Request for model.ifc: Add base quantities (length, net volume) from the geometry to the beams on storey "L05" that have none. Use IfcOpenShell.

First a look at what the model holds.

```python
import ifcopenshell
import ifcopenshell.util.element
import ifcopenshell.util.unit

model = ifcopenshell.open("model.ifc")
print(model.schema)
for unit_type in ("LENGTHUNIT", "AREAUNIT", "VOLUMEUNIT"):
    print(unit_type, ifcopenshell.util.unit.calculate_unit_scale(model, unit_type))
storey = next(s for s in model.by_type("IfcBuildingStorey") if s.Name == "L05")
beams = [e for e in ifcopenshell.util.element.get_decomposition(storey) if e.is_a("IfcBeam")]
for e in sorted(beams, key=lambda e: e.id()):
    print(e.id(), e.is_a(), e.Name, list(ifcopenshell.util.element.get_psets(e, qtos_only=True)), sep=" | ")
```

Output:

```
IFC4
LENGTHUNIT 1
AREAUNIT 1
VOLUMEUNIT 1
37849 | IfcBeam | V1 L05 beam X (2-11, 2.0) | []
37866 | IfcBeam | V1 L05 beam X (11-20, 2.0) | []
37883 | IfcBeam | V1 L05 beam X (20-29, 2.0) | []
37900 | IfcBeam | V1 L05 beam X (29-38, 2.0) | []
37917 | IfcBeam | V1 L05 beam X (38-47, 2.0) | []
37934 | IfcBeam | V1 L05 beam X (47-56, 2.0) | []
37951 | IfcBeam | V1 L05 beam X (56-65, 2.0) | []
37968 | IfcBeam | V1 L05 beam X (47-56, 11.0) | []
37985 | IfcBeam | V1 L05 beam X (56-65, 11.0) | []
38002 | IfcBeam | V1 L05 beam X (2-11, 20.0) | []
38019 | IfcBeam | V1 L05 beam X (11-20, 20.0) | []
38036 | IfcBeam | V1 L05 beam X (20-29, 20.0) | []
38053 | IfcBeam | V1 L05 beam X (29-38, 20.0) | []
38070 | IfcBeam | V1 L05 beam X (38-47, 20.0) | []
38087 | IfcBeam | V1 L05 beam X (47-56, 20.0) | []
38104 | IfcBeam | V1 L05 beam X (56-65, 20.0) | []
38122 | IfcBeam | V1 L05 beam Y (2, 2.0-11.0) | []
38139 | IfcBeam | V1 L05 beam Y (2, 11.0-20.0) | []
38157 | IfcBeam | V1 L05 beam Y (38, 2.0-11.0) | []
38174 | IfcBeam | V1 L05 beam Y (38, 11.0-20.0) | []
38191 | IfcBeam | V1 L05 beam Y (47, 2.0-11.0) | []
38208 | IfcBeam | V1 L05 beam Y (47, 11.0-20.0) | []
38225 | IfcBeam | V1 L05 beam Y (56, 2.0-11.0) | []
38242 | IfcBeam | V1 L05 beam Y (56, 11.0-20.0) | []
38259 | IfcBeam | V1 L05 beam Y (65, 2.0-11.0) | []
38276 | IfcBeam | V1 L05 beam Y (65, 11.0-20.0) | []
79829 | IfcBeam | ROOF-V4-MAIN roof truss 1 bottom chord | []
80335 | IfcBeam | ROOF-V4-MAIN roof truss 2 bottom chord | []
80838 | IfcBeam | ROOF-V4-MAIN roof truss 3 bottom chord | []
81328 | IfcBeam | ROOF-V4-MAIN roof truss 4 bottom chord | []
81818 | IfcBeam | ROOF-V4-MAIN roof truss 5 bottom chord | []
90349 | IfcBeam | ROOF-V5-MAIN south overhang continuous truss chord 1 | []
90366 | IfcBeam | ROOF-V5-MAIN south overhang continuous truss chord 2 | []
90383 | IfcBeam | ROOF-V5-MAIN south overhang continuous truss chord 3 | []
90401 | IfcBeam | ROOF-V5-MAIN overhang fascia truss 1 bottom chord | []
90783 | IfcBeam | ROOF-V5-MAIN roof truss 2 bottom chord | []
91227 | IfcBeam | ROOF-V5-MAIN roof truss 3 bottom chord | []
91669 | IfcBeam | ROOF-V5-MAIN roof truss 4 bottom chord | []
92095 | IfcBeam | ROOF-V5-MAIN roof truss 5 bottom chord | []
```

```python
import ifcopenshell
import ifcopenshell.api.pset
import ifcopenshell.geom
import ifcopenshell.util.element
import ifcopenshell.util.shape
import ifcopenshell.util.unit

model = ifcopenshell.open("model.ifc")
unit_scale = ifcopenshell.util.unit.calculate_unit_scale(model)
volume_scale = ifcopenshell.util.unit.calculate_unit_scale(model, "VOLUMEUNIT")
settings = ifcopenshell.geom.settings()

storey = next(s for s in model.by_type("IfcBuildingStorey") if s.Name == "L05")
beams = [e for e in ifcopenshell.util.element.get_decomposition(storey) if e.is_a("IfcBeam")]

for e in sorted(beams, key=lambda e: e.id()):
    if ifcopenshell.util.element.get_psets(e, qtos_only=True, should_inherit=False):
        continue
    # Geometry comes back in metres, in the element's own axes.
    shape = ifcopenshell.geom.create_shape(settings, e)
    values = {
        "Length": ifcopenshell.util.shape.get_max_xyz(shape.geometry) / unit_scale,
        "NetVolume": ifcopenshell.util.shape.get_volume(shape.geometry) / volume_scale,
    }
    qto = ifcopenshell.api.pset.add_qto(model, product=e, name="Qto_BeamBaseQuantities")
    ifcopenshell.api.pset.edit_qto(model, qto=qto, properties=values)
    print(e.id(), {k: round(v, 3) for k, v in values.items()})

model.write("model-out.ifc")
```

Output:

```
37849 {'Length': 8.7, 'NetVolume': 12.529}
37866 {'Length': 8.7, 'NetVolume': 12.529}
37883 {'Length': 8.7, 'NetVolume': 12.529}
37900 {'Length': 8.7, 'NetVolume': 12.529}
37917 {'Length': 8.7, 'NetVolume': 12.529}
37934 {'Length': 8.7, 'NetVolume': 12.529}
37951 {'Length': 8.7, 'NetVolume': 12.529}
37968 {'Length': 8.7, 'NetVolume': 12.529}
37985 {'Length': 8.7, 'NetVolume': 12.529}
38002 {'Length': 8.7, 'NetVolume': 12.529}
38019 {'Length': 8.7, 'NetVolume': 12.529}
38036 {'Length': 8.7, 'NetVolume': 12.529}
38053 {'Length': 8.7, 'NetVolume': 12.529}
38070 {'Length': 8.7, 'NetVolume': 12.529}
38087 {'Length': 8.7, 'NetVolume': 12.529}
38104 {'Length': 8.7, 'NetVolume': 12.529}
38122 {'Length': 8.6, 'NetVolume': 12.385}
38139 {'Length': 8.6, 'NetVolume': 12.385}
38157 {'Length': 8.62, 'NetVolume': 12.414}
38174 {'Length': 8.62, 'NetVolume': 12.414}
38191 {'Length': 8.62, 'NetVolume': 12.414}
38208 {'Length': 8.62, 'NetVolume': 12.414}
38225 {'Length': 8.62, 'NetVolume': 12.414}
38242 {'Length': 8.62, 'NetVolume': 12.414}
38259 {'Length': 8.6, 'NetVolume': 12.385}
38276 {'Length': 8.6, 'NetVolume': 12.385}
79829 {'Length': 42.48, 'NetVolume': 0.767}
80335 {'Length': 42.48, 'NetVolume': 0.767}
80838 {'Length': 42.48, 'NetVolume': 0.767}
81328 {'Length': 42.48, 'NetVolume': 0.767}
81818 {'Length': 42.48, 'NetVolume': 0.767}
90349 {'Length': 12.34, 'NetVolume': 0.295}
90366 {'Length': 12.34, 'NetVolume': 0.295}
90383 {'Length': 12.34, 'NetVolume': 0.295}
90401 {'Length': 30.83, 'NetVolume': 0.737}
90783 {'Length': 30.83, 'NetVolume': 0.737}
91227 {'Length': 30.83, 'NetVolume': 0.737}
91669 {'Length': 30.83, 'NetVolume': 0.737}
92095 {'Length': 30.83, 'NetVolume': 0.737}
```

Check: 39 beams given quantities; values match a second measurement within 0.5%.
